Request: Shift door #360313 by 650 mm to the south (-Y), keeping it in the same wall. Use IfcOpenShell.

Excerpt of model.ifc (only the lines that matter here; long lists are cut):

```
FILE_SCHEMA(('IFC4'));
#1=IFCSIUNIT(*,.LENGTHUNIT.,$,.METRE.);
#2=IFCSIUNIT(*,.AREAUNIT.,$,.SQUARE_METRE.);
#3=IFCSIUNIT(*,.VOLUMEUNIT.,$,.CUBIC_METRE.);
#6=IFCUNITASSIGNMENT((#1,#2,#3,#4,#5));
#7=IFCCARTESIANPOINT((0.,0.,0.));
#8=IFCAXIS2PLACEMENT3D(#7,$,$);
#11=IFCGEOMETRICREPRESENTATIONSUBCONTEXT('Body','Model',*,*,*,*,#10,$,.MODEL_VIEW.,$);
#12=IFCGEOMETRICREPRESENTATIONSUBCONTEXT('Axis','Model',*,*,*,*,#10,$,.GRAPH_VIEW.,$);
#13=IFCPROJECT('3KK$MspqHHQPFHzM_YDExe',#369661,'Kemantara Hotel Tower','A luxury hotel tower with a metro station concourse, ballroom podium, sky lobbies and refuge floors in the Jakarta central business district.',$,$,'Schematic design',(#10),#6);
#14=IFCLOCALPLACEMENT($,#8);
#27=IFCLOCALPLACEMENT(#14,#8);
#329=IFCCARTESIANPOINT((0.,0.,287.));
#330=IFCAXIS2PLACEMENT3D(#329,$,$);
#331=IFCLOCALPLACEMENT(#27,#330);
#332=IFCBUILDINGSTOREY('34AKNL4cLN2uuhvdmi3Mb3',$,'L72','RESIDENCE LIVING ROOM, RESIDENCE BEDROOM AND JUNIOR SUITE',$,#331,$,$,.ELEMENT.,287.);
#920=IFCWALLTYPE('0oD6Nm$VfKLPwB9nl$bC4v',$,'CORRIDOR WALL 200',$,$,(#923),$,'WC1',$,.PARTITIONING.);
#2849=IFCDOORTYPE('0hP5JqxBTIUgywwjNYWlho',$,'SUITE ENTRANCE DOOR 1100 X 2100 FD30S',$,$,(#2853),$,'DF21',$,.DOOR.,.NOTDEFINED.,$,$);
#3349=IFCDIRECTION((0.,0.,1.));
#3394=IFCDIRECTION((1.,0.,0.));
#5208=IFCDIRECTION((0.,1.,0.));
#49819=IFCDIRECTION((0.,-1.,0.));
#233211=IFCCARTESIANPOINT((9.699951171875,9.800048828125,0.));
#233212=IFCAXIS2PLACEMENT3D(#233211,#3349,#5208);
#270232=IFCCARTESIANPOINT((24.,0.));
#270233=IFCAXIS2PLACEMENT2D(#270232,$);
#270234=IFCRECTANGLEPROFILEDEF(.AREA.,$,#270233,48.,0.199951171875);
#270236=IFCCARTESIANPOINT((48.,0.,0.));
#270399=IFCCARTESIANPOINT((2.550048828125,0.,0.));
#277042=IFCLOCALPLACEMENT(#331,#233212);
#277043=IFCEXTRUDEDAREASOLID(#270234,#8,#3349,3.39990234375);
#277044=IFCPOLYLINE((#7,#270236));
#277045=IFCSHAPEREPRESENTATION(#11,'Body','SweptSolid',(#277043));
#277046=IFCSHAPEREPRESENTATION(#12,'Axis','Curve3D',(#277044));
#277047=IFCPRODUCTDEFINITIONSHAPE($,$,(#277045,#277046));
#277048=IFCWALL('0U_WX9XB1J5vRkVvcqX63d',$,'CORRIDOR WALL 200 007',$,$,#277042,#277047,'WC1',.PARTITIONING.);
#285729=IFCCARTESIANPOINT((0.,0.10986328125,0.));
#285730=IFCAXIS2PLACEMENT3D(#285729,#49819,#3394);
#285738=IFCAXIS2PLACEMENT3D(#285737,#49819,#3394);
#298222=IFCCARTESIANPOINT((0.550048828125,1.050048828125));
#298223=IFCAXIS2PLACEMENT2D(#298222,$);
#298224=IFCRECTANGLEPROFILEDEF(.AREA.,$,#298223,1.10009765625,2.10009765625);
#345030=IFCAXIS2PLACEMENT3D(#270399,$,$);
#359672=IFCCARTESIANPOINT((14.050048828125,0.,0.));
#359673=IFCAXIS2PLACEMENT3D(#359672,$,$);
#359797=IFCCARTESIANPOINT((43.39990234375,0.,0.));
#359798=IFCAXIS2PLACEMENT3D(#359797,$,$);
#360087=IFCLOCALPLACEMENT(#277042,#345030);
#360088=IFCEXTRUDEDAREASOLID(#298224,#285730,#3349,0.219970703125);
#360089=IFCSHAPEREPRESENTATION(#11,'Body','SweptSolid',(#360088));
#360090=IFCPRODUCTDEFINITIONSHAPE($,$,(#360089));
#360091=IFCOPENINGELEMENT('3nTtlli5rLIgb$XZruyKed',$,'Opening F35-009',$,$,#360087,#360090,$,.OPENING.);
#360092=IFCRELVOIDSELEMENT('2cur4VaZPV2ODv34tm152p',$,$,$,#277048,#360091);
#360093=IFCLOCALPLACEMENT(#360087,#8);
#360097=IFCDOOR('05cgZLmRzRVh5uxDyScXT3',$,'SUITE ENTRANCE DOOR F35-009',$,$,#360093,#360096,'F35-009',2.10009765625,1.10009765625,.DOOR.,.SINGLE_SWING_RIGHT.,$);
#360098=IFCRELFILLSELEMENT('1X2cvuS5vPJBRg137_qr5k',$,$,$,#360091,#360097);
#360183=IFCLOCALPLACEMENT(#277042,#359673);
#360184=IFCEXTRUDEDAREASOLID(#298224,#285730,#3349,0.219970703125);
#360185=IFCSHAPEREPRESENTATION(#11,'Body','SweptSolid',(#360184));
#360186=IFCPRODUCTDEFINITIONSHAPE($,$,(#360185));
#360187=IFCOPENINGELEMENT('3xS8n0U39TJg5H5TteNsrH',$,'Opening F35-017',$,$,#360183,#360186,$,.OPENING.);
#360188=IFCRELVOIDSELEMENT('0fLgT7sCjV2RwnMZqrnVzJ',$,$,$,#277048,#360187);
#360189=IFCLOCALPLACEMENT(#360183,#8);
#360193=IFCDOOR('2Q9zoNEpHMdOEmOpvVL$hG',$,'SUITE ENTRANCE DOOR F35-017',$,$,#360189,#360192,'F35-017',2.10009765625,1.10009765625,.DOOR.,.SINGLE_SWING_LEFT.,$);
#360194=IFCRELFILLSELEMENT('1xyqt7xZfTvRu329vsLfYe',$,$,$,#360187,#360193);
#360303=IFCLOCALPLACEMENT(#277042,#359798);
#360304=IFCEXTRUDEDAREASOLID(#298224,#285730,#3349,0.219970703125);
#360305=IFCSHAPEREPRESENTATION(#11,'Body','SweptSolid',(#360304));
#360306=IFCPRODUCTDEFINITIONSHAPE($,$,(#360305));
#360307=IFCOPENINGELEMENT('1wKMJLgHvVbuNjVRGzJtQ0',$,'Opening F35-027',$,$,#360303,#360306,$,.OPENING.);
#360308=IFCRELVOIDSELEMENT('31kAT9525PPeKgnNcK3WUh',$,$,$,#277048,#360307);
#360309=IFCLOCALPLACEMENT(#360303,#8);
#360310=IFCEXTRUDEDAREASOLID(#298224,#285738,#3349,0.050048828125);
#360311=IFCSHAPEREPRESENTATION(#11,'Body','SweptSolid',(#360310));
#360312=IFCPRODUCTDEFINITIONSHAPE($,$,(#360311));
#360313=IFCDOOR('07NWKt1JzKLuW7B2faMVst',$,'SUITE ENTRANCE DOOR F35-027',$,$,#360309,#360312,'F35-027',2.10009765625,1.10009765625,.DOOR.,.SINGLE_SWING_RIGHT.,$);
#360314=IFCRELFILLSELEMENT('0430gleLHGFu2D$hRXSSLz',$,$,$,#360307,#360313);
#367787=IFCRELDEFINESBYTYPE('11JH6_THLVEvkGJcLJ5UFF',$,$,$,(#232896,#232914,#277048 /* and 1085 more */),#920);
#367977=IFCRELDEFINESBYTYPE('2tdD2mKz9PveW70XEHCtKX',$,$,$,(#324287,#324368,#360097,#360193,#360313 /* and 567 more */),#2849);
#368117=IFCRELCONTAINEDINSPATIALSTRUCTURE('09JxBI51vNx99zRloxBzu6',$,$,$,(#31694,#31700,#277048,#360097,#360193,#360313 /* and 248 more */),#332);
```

```python
import ifcopenshell
import ifcopenshell.api.geometry
import ifcopenshell.util.placement

model = ifcopenshell.open("model.ifc")

door = model.by_id(360313)
opening = door.FillsVoids[0].RelatingOpeningElement
wall = opening.VoidsElements[0].RelatingBuildingElement

wall_matrix = ifcopenshell.util.placement.get_local_placement(wall.ObjectPlacement)
shift = wall_matrix[:3, 0] * -0.65
before = ifcopenshell.util.placement.get_local_placement(door.ObjectPlacement)[:3, 3].copy()

# The door is placed relative to its opening, so it follows when the opening moves.
matrix = ifcopenshell.util.placement.get_local_placement(opening.ObjectPlacement)
matrix[:3, 3] += shift
ifcopenshell.api.geometry.edit_object_placement(
    model, product=opening, matrix=matrix, is_si=False, should_transform_children=True
)

after = ifcopenshell.util.placement.get_local_placement(door.ObjectPlacement)[:3, 3]
print("door moved by", (after - before).round(3) + 0.0)

model.write("model_rev.ifc")
```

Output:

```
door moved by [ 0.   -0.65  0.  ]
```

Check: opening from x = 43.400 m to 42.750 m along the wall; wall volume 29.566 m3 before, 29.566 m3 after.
